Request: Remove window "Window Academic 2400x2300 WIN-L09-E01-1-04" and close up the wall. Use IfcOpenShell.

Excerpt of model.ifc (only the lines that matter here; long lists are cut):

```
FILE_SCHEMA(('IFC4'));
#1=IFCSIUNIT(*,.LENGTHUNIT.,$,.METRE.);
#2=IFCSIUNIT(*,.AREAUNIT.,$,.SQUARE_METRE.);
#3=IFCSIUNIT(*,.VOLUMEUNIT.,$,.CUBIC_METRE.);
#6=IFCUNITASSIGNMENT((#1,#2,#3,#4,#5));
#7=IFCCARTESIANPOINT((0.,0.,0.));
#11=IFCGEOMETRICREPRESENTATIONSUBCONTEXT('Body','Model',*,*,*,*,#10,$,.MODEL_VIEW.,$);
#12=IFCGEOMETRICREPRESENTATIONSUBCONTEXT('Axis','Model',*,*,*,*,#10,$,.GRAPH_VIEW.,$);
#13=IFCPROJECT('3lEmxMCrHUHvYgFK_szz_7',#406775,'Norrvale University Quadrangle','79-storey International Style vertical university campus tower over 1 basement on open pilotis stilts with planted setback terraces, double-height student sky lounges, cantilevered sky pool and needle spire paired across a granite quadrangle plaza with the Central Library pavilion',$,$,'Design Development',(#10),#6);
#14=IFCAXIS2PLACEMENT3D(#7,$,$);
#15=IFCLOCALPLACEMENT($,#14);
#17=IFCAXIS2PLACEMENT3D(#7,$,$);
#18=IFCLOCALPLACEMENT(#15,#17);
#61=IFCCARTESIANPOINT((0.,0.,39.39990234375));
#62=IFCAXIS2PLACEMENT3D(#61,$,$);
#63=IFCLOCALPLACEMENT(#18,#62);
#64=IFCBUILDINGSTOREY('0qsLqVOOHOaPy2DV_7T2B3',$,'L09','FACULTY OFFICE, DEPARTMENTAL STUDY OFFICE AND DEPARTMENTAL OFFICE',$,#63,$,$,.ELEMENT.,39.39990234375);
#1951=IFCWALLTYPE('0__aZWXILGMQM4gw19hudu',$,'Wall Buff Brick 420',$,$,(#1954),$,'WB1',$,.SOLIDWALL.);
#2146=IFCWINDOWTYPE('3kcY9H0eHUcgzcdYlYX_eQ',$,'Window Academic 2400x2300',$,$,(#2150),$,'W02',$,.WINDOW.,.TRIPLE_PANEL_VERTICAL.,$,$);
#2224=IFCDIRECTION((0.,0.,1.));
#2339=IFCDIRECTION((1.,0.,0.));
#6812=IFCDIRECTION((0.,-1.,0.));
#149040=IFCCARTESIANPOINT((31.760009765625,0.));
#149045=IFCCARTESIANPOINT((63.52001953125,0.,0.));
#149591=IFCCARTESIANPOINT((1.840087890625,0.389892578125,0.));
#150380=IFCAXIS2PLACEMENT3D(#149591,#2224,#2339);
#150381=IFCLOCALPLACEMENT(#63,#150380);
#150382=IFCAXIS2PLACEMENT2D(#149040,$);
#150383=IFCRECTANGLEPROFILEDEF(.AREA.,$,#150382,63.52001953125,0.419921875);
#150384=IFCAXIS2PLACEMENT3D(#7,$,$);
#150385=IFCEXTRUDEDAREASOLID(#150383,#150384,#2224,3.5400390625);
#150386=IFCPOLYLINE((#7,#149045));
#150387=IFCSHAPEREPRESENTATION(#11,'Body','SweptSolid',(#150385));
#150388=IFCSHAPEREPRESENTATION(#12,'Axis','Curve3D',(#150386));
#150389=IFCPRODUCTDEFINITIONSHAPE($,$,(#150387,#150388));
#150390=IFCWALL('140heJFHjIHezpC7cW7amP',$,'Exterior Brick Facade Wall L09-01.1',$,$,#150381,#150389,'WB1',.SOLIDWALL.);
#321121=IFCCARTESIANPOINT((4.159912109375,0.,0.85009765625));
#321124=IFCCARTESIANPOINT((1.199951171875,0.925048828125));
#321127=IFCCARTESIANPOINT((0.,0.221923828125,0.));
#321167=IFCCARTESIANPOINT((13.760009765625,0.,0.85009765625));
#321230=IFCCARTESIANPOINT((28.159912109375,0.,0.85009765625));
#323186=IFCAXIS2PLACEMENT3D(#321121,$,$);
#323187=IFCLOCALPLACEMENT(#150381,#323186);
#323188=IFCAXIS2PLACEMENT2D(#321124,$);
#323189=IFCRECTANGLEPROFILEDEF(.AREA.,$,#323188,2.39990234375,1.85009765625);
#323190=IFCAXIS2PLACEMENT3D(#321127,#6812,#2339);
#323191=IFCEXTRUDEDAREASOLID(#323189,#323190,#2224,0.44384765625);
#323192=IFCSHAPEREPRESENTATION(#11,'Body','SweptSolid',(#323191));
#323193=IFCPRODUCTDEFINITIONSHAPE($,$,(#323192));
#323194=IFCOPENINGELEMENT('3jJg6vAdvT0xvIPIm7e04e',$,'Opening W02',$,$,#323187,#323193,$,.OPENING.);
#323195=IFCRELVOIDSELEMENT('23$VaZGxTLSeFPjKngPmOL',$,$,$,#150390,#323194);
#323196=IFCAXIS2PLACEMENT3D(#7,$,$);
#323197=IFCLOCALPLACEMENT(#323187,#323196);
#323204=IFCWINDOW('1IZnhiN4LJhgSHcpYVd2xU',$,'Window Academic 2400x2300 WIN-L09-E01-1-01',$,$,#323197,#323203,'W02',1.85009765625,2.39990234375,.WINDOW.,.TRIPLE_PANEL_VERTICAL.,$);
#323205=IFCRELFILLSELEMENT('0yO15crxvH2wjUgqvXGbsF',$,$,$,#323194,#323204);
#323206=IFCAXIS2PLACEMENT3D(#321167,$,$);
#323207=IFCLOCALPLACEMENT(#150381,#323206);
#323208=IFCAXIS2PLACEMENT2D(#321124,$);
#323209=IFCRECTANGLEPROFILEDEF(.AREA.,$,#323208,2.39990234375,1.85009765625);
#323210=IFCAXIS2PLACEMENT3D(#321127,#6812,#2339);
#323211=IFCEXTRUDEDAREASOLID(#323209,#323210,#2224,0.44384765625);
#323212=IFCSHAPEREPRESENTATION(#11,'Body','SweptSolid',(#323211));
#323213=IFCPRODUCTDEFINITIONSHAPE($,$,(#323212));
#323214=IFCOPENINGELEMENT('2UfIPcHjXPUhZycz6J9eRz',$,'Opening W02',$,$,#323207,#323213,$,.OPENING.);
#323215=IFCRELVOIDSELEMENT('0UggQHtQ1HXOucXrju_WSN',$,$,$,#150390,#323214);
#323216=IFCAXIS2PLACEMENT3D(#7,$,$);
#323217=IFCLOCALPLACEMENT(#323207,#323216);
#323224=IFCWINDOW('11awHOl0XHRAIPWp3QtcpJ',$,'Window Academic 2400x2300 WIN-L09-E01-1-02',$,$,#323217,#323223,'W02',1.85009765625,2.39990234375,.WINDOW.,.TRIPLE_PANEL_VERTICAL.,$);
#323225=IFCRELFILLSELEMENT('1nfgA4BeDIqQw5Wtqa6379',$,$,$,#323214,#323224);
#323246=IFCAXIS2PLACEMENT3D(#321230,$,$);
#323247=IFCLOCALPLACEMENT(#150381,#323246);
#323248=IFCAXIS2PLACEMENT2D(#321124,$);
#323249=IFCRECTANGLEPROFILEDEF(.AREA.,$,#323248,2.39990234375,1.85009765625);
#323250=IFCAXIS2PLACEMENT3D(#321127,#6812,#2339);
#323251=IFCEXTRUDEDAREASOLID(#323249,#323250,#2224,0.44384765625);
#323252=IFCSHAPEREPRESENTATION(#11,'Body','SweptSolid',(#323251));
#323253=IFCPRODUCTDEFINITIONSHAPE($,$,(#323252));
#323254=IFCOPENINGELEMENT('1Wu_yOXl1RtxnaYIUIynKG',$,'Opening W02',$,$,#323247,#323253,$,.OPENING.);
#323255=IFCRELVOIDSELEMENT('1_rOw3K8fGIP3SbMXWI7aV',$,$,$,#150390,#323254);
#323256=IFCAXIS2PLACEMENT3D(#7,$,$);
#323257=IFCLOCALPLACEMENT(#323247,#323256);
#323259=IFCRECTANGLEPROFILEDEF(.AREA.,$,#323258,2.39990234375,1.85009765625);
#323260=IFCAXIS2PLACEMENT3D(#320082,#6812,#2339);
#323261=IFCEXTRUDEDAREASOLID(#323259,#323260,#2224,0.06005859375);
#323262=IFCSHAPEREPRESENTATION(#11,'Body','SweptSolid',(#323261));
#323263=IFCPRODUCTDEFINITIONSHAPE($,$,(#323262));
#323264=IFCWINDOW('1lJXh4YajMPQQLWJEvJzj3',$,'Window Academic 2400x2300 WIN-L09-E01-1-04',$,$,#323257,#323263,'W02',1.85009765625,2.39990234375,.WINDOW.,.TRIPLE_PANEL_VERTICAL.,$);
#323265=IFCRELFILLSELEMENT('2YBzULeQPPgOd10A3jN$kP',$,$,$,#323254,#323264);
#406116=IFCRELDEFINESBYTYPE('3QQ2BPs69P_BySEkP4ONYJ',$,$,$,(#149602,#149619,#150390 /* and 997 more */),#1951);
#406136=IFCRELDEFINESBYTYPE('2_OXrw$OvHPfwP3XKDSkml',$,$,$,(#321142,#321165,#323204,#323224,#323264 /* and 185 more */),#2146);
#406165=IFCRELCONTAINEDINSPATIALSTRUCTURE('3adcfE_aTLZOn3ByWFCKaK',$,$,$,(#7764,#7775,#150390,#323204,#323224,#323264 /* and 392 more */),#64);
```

```python
import ifcopenshell
import ifcopenshell.api.feature
import ifcopenshell.api.root
import ifcopenshell.geom
import ifcopenshell.util.shape

model = ifcopenshell.open("model.ifc")
settings = ifcopenshell.geom.settings()


def volume(element):
    """Net volume in cubic metres, openings subtracted."""
    shape = ifcopenshell.geom.create_shape(settings, element)
    return ifcopenshell.util.shape.get_volume(shape.geometry)


window = model.by_guid("1lJXh4YajMPQQLWJEvJzj3")
opening = window.FillsVoids[0].RelatingOpeningElement
wall = opening.VoidsElements[0].RelatingBuildingElement
before = volume(wall)

ifcopenshell.api.root.remove_product(model, product=window)
ifcopenshell.api.feature.remove_feature(model, feature=opening)

after = volume(wall)

print(f"wall volume {before:.3f} -> {after:.3f} m3")

model.write("model_edited.ifc")
```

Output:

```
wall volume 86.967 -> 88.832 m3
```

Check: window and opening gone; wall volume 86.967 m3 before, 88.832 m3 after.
